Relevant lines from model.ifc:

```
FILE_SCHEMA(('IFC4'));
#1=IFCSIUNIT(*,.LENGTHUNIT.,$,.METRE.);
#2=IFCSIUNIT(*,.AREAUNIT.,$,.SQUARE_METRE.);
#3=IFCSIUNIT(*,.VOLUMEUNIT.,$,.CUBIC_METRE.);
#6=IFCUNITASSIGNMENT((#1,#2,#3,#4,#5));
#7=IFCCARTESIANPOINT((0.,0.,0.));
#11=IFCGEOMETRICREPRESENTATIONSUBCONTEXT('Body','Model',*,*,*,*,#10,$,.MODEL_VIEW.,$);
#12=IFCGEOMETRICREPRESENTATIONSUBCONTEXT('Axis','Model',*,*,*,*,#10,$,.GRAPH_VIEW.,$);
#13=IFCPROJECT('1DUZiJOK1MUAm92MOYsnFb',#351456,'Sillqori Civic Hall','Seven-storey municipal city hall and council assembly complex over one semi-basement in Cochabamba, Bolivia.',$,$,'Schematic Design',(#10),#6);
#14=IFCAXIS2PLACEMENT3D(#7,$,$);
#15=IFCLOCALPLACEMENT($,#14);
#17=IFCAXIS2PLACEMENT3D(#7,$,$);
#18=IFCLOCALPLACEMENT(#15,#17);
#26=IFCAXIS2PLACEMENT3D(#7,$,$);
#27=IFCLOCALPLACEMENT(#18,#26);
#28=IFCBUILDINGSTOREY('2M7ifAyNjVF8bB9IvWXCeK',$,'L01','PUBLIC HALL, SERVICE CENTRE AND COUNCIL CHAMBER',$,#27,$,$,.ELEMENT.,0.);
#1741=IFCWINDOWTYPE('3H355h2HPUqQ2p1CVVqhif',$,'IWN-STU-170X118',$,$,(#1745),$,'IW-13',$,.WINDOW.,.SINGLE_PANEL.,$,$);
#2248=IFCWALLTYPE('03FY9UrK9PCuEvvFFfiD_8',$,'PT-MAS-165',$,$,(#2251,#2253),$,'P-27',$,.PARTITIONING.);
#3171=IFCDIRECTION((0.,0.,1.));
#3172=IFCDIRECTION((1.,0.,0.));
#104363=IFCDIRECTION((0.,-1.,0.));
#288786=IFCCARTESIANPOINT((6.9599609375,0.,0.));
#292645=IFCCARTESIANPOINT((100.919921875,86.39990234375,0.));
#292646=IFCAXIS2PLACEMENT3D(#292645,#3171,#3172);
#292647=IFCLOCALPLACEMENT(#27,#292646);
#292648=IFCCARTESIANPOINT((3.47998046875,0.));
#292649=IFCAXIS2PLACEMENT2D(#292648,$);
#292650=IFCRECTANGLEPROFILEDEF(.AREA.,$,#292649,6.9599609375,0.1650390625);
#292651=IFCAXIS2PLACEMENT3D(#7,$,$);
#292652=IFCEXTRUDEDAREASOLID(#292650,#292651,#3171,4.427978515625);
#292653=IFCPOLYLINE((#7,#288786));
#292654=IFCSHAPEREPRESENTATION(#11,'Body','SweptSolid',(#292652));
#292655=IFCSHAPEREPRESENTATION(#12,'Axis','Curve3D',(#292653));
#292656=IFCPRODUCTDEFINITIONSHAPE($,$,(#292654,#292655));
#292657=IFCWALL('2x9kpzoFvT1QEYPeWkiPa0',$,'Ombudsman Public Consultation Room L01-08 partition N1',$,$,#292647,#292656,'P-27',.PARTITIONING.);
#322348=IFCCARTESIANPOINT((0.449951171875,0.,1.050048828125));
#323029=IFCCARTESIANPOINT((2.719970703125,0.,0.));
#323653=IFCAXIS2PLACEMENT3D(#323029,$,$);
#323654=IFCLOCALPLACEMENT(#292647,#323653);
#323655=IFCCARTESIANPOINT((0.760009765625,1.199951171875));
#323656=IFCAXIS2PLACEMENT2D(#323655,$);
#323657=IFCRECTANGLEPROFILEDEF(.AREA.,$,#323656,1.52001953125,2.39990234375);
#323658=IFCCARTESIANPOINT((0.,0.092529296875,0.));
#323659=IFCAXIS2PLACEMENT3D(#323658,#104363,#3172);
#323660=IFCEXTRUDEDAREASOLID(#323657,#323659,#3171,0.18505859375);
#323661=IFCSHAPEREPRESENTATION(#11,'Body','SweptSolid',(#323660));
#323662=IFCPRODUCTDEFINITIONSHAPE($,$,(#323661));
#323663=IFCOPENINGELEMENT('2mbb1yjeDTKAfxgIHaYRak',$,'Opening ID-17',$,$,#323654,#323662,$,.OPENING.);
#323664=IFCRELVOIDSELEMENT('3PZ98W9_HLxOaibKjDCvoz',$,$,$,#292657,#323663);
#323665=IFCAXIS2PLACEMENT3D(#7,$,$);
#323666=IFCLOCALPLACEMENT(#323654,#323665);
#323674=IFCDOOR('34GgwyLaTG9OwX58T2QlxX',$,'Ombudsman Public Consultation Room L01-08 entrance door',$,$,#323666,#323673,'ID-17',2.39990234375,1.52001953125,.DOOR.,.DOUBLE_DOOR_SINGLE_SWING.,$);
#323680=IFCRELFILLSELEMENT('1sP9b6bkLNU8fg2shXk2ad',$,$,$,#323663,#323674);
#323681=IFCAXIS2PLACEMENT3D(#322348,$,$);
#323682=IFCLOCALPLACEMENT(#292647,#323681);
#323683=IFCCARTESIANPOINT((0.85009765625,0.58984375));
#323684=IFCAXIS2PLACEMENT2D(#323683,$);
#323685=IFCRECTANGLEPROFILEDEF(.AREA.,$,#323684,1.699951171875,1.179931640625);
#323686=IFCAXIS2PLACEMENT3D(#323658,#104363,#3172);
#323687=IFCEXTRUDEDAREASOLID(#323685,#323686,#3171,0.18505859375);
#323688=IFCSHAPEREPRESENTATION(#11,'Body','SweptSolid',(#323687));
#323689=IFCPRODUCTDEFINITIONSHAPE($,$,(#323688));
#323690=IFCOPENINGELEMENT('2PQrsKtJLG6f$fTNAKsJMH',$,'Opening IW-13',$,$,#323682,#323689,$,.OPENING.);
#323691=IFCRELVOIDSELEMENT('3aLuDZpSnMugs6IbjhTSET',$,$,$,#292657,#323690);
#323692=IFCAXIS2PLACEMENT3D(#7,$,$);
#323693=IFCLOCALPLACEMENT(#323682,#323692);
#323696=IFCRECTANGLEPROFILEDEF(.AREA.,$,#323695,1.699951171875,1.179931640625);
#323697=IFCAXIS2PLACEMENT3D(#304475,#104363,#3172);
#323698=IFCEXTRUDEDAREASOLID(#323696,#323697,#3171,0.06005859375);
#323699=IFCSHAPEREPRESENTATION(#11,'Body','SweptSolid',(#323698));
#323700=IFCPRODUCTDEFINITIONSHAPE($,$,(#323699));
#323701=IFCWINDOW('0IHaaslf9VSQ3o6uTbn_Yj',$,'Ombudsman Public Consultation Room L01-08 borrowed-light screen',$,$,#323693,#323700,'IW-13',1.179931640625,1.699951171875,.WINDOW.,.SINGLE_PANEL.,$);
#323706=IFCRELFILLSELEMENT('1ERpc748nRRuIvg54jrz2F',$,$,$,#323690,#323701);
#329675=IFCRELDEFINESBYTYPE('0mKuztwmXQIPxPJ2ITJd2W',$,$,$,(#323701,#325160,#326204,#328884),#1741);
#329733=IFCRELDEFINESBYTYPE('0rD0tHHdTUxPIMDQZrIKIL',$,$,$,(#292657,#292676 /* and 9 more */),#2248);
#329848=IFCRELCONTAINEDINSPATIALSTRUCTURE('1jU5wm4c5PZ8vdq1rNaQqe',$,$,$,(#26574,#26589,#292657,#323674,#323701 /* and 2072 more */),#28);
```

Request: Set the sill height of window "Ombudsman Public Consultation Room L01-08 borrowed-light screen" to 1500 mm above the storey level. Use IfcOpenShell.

```python
import numpy as np
import ifcopenshell
import ifcopenshell.api.geometry
import ifcopenshell.geom
import ifcopenshell.util.element
import ifcopenshell.util.placement
import ifcopenshell.util.shape
import ifcopenshell.util.unit

model = ifcopenshell.open("model.ifc")
unit_scale = ifcopenshell.util.unit.calculate_unit_scale(model)

window = model.by_guid("0IHaaslf9VSQ3o6uTbn_Yj")
opening = window.FillsVoids[0].RelatingOpeningElement
storey = ifcopenshell.util.element.get_container(window, ifc_class="IfcBuildingStorey")
level = ifcopenshell.util.placement.get_local_placement(storey.ObjectPlacement)[2, 3]

# The opening's origin need not be at the sill, so measure its lowest point.
shape = ifcopenshell.geom.create_shape(ifcopenshell.geom.settings(), opening)
bottom = ifcopenshell.util.shape.get_shape_bottom_elevation(shape, shape.geometry) / unit_scale
dz = level + 1.5 / unit_scale - bottom

shift = np.array([0.0, 0.0, dz])
# The window is placed relative to its opening, so it follows when the opening moves.
matrix = ifcopenshell.util.placement.get_local_placement(opening.ObjectPlacement)
matrix[:3, 3] += shift
ifcopenshell.api.geometry.edit_object_placement(
    model, product=opening, matrix=matrix, is_si=False, should_transform_children=True
)

print(f"moved by {dz * unit_scale:+.3f} m")

model.write("model_v2.ifc")
```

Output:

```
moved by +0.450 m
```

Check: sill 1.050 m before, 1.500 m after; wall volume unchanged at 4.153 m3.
